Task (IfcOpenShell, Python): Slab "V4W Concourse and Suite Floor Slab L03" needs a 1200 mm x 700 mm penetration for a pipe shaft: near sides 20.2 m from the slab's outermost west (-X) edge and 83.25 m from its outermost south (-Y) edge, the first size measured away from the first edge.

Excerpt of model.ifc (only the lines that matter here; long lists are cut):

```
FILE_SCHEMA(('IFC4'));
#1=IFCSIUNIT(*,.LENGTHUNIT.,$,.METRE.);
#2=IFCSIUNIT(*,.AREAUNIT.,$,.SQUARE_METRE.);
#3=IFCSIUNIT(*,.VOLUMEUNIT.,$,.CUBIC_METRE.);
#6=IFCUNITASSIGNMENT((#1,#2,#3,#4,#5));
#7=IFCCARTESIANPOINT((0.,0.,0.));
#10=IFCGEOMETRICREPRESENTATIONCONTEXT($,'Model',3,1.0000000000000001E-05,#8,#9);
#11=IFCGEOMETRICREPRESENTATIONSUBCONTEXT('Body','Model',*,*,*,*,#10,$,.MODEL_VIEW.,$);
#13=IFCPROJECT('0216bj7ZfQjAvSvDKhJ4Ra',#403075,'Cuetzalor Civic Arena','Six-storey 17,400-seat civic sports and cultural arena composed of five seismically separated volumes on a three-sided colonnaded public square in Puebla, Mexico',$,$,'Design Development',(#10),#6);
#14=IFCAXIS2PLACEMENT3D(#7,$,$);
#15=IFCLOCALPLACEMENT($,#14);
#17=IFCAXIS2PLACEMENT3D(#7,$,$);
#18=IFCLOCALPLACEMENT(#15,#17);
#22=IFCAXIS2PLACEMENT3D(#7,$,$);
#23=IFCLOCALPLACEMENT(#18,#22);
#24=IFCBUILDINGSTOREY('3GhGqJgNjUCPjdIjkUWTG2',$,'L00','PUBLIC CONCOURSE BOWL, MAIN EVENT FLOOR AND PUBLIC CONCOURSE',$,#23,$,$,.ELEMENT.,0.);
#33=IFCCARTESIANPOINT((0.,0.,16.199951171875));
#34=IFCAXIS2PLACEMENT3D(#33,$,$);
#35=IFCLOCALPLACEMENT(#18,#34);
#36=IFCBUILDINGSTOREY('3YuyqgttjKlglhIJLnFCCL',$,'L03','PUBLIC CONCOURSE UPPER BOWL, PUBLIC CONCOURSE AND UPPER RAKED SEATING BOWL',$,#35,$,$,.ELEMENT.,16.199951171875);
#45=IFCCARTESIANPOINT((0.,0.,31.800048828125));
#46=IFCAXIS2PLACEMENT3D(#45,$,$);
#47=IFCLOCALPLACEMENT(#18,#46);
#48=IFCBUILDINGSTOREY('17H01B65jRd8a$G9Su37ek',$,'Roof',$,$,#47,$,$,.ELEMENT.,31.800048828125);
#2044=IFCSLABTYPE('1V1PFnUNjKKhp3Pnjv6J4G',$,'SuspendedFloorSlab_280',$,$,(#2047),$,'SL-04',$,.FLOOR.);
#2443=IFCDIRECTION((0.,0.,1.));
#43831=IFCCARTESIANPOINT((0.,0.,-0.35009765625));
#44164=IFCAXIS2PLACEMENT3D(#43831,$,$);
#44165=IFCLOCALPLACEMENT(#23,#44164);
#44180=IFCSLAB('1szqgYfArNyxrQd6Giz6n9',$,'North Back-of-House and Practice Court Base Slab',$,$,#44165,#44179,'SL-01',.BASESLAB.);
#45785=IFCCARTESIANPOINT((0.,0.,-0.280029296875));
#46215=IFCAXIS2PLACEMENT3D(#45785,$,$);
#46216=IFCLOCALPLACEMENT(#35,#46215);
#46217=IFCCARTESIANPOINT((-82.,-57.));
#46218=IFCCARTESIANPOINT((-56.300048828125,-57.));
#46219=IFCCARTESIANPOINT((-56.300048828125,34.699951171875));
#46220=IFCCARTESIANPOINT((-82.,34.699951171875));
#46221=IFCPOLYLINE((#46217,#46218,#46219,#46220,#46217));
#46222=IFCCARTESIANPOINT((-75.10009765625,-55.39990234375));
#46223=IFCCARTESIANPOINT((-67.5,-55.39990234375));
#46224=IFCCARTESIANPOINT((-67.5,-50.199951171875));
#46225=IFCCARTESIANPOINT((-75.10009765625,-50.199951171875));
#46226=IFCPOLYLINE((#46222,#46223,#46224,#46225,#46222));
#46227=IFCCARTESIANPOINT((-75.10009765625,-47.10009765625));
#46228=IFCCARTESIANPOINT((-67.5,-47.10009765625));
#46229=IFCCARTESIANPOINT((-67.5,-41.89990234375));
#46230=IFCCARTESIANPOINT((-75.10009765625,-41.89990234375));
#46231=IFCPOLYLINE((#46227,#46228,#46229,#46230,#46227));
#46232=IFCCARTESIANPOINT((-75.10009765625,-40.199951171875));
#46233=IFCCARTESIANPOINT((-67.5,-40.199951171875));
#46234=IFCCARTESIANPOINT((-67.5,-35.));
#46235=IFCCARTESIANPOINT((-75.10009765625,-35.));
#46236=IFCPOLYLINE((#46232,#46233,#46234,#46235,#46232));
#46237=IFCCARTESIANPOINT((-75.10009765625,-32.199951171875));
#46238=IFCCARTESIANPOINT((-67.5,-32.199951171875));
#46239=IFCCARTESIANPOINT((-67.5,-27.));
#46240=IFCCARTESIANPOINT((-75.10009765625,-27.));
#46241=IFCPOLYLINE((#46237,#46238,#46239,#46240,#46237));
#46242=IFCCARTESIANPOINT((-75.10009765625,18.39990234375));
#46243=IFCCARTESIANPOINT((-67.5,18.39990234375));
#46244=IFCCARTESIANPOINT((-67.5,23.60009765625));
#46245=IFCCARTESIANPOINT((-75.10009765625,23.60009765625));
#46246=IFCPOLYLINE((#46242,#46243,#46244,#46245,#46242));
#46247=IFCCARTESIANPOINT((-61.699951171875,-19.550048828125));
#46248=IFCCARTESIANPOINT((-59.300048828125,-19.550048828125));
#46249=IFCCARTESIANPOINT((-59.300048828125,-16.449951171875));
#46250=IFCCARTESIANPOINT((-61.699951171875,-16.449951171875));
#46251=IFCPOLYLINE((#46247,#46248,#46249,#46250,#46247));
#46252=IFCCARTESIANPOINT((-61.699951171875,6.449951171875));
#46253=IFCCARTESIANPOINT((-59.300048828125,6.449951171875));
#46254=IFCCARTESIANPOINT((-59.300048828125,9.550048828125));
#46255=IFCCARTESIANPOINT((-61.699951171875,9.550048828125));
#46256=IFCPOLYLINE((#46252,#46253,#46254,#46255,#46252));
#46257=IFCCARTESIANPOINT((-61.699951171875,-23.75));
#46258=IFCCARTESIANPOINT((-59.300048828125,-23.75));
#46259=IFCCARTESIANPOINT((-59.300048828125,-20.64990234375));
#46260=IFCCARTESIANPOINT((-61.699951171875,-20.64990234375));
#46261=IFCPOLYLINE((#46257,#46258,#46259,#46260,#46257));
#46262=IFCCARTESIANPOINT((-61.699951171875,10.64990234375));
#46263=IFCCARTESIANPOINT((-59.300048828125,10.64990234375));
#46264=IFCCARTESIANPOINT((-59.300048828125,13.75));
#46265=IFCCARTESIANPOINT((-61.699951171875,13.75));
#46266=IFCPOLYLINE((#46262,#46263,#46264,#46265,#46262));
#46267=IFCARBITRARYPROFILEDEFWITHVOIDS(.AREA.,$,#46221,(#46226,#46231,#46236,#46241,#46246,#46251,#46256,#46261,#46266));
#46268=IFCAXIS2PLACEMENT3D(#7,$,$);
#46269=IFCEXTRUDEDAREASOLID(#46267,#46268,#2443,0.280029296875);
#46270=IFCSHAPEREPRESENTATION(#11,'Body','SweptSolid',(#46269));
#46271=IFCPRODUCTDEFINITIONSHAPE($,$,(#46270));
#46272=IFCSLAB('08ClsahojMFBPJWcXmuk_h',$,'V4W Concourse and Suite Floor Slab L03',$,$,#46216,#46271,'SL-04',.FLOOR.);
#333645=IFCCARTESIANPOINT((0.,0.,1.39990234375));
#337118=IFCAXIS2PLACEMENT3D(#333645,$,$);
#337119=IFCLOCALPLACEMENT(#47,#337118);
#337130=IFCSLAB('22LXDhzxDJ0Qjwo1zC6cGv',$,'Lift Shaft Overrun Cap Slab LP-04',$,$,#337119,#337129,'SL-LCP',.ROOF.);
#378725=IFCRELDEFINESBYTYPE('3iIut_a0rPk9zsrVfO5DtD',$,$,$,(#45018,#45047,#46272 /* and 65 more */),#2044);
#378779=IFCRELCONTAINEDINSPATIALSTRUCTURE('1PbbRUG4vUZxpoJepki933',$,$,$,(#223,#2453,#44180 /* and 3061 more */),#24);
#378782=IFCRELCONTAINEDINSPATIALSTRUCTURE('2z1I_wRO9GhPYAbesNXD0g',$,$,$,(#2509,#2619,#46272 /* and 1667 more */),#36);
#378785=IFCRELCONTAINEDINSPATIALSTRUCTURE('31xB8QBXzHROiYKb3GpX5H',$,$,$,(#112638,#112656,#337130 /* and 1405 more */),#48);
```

```python
import numpy as np
import ifcopenshell
import ifcopenshell.api.feature
import ifcopenshell.api.geometry
import ifcopenshell.api.root
import ifcopenshell.geom
import ifcopenshell.util.placement
import ifcopenshell.util.representation
import ifcopenshell.util.shape
import ifcopenshell.util.unit

model = ifcopenshell.open("model.ifc")
unit_scale = ifcopenshell.util.unit.calculate_unit_scale(model)
settings = ifcopenshell.geom.settings()


def volume(element):
    """Net volume in cubic metres, openings subtracted."""
    shape = ifcopenshell.geom.create_shape(settings, element)
    return ifcopenshell.util.shape.get_volume(shape.geometry)


slab = model.by_id(46272)
before = volume(slab)

# Extent in the slab's own axes, in metres. The edges named are its -X and -Y sides.
slab_shape = ifcopenshell.geom.create_shape(settings, slab)
vertices = ifcopenshell.util.shape.get_vertices(slab_shape.geometry)
x_min, y_min, bottom = vertices.min(axis=0)
top = vertices[:, 2].max()

opening = ifcopenshell.api.root.create_entity(model, ifc_class="IfcOpeningElement", name="Pipe shaft opening", predefined_type="OPENING")
context = ifcopenshell.util.representation.get_context(model, "Model", "Body", "MODEL_VIEW")
width, depth = 1.2, 0.7
outline = [(0.0, 0.0), (width, 0.0), (width, depth), (0.0, depth), (0.0, 0.0)]
# Overshoot both faces by 50 mm so the cut is clean.
shape = ifcopenshell.api.geometry.add_slab_representation(
    model, context=context, depth=top - bottom + 0.1, polyline=outline
)
ifcopenshell.api.geometry.assign_representation(model, product=opening, representation=shape)

matrix = ifcopenshell.util.placement.get_local_placement(slab.ObjectPlacement)
matrix[:, 3] = matrix @ np.append(np.array([x_min + 20.2, y_min + 83.25, bottom - 0.05]) / unit_scale, 1.0)
ifcopenshell.api.geometry.edit_object_placement(model, product=opening, matrix=matrix, is_si=False)
ifcopenshell.api.feature.add_feature(model, feature=opening, element=slab)

after = volume(slab)

print(f"slab volume {before:.3f} -> {after:.3f} m3")

model.write("model_edited.ifc")
```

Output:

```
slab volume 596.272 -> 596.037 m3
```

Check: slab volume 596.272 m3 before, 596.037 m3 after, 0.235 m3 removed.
